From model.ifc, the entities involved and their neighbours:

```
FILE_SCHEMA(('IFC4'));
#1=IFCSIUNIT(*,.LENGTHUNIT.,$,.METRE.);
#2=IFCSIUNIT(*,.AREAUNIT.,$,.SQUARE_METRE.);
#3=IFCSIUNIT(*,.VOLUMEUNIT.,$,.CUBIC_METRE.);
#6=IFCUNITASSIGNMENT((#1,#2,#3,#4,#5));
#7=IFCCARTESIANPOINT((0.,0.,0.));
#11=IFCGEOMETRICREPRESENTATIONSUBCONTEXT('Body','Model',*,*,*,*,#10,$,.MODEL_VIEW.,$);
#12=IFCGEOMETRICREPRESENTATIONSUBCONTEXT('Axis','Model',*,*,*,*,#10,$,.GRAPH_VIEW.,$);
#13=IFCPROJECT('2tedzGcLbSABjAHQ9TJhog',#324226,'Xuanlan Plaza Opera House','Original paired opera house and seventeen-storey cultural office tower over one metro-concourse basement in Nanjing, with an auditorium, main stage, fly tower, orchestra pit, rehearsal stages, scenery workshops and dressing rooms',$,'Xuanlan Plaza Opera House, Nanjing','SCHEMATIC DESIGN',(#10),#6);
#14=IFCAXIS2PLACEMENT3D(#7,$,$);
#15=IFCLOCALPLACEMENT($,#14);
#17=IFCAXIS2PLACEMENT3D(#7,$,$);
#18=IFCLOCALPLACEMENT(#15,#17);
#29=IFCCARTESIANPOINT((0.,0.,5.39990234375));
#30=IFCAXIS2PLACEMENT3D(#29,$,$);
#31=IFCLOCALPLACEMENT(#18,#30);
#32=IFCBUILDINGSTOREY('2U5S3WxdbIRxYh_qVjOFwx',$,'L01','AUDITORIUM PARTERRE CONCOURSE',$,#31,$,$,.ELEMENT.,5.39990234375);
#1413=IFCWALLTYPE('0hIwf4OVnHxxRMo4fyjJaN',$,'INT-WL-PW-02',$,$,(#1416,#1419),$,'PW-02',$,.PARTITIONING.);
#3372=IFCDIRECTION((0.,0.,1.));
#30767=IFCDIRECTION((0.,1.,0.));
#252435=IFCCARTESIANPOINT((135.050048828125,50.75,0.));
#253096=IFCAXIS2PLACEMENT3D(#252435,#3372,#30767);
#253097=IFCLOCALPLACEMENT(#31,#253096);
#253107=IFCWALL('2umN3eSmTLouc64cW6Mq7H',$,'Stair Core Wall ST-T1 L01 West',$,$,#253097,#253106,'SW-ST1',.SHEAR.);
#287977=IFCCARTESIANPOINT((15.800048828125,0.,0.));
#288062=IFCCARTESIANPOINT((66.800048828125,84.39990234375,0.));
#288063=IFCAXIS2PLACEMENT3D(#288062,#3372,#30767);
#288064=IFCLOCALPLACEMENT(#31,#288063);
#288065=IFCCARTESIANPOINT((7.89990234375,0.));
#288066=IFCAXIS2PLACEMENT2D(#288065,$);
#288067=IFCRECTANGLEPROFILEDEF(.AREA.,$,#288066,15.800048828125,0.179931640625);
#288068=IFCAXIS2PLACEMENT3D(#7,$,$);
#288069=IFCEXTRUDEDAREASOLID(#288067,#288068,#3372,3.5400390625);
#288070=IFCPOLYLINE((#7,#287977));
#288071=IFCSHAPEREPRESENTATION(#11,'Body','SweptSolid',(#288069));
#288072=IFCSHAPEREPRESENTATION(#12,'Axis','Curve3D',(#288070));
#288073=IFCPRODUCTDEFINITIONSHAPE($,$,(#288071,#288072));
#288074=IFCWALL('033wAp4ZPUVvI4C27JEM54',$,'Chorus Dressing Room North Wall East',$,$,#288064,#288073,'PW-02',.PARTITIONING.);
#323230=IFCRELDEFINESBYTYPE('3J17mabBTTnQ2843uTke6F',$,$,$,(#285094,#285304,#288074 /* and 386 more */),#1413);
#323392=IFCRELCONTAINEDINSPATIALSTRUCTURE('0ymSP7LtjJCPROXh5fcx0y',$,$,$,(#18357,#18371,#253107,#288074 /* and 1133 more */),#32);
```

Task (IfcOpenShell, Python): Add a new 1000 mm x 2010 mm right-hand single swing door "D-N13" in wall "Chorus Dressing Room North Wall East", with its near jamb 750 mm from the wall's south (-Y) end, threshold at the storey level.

```python
import numpy as np
import ifcopenshell
import ifcopenshell.api.feature
import ifcopenshell.api.geometry
import ifcopenshell.api.root
import ifcopenshell.api.spatial
import ifcopenshell.geom
import ifcopenshell.util.element
import ifcopenshell.util.placement
import ifcopenshell.util.representation
import ifcopenshell.util.shape
import ifcopenshell.util.unit

model = ifcopenshell.open("model.ifc")
unit_scale = ifcopenshell.util.unit.calculate_unit_scale(model)
settings = ifcopenshell.geom.settings()


def volume(element):
    """Net volume in cubic metres, openings subtracted."""
    shape = ifcopenshell.geom.create_shape(settings, element)
    return ifcopenshell.util.shape.get_volume(shape.geometry)


wall = model.by_guid("033wAp4ZPUVvI4C27JEM54")
storey = ifcopenshell.util.element.get_container(wall, ifc_class="IfcBuildingStorey")
context = ifcopenshell.util.representation.get_context(model, "Model", "Body", "MODEL_VIEW")
before = volume(wall)

width, height, from_end, sill = 1, 2.01, 0.75, 0.0  # metres

# The wall runs along its own X axis, and the end named is its -X end.
wall_shape = ifcopenshell.geom.create_shape(settings, wall)
x, y, z = ifcopenshell.util.shape.get_vertices(wall_shape.geometry).T
start = x.min() + from_end
face, thickness = float(y.min()), float(y.max() - y.min())
wall_matrix = ifcopenshell.util.placement.get_local_placement(wall.ObjectPlacement)
level = ifcopenshell.util.placement.get_local_placement(storey.ObjectPlacement)[2, 3]


def in_wall(x, y):
    """Placement at x, y metres in the wall's axes, at sill height."""
    matrix = wall_matrix.copy()
    matrix[:, 3] = wall_matrix @ np.array([x / unit_scale, y / unit_scale, 0.0, 1.0])
    matrix[2, 3] = level + sill / unit_scale
    return matrix


# Opening: a box that overshoots both wall faces by 50 mm.
opening = ifcopenshell.api.root.create_entity(model, ifc_class="IfcOpeningElement", predefined_type="OPENING")
box = ifcopenshell.api.geometry.add_wall_representation(
    model, context=context, length=width, height=height, thickness=thickness + 0.1
)
ifcopenshell.api.geometry.assign_representation(model, product=opening, representation=box)
ifcopenshell.api.geometry.edit_object_placement(model, product=opening, matrix=in_wall(start, face - 0.05), is_si=False)
ifcopenshell.api.feature.add_feature(model, feature=opening, element=wall)

door = ifcopenshell.api.root.create_entity(model, ifc_class="IfcDoor", name="D-N13", predefined_type="DOOR")
door.OverallWidth, door.OverallHeight = width / unit_scale, height / unit_scale
door.OperationType = "SINGLE_SWING_RIGHT"
body = ifcopenshell.api.geometry.add_door_representation(
    model,
    context=context,
    overall_width=door.OverallWidth,
    overall_height=door.OverallHeight,
    operation_type="SINGLE_SWING_RIGHT",
    lining_properties={"LiningDepth": thickness / unit_scale, "ThresholdDepth": thickness / unit_scale},
)
ifcopenshell.api.geometry.assign_representation(model, product=door, representation=body)
ifcopenshell.api.spatial.assign_container(model, products=[door], relating_structure=storey)
ifcopenshell.api.feature.add_filling(model, opening=opening, element=door)

# The lining spans the wall, so the door starts at the wall face.
ifcopenshell.api.geometry.edit_object_placement(model, product=door, matrix=in_wall(start, face), is_si=False)

after = volume(wall)

print(f"wall volume {before:.3f} -> {after:.3f} m3")

model.write("model_edited.ifc")
```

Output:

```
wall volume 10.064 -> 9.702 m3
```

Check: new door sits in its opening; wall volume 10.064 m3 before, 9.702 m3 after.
